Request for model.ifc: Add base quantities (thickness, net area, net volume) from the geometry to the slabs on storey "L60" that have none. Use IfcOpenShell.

First a look at what the model holds.

```python
import ifcopenshell
import ifcopenshell.util.element
import ifcopenshell.util.unit

model = ifcopenshell.open("model.ifc")
print(model.schema)
for unit_type in ("LENGTHUNIT", "AREAUNIT", "VOLUMEUNIT"):
    print(unit_type, ifcopenshell.util.unit.calculate_unit_scale(model, unit_type))
storey = next(s for s in model.by_type("IfcBuildingStorey") if s.Name == "L60")
slabs = [e for e in ifcopenshell.util.element.get_decomposition(storey) if e.is_a("IfcSlab")]
for e in sorted(slabs, key=lambda e: e.id()):
    print(e.id(), e.is_a(), e.Name, list(ifcopenshell.util.element.get_psets(e, qtos_only=True)), sep=" | ")
```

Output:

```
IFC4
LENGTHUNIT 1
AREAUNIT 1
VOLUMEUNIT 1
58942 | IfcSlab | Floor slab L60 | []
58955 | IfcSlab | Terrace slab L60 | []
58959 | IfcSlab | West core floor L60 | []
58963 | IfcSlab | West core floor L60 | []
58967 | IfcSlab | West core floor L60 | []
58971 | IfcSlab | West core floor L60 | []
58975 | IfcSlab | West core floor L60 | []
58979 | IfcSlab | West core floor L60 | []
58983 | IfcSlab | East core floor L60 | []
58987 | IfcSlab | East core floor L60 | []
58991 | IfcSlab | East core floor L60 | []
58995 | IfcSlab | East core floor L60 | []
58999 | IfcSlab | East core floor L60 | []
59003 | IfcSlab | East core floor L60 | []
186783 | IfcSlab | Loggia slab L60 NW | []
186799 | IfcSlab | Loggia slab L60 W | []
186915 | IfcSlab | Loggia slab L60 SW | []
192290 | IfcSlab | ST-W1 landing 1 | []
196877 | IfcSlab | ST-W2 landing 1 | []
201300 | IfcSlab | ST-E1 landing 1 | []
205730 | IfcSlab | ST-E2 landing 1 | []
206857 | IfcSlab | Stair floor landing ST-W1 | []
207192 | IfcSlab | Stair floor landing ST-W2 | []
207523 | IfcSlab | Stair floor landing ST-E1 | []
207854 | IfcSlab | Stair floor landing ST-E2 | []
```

```python
import ifcopenshell
import ifcopenshell.api.pset
import ifcopenshell.geom
import ifcopenshell.util.element
import ifcopenshell.util.shape
import ifcopenshell.util.unit

model = ifcopenshell.open("model.ifc")
unit_scale = ifcopenshell.util.unit.calculate_unit_scale(model)
area_scale = ifcopenshell.util.unit.calculate_unit_scale(model, "AREAUNIT")
volume_scale = ifcopenshell.util.unit.calculate_unit_scale(model, "VOLUMEUNIT")
settings = ifcopenshell.geom.settings()

storey = next(s for s in model.by_type("IfcBuildingStorey") if s.Name == "L60")
slabs = [e for e in ifcopenshell.util.element.get_decomposition(storey) if e.is_a("IfcSlab")]

for e in sorted(slabs, key=lambda e: e.id()):
    if ifcopenshell.util.element.get_psets(e, qtos_only=True, should_inherit=False):
        continue
    # Geometry comes back in metres, in the element's own axes.
    shape = ifcopenshell.geom.create_shape(settings, e)
    values = {
        "Width": ifcopenshell.util.shape.get_z(shape.geometry) / unit_scale,
        "NetArea": ifcopenshell.util.shape.get_footprint_area(shape.geometry) / area_scale,
        "NetVolume": ifcopenshell.util.shape.get_volume(shape.geometry) / volume_scale,
    }
    qto = ifcopenshell.api.pset.add_qto(model, product=e, name="Qto_SlabBaseQuantities")
    ifcopenshell.api.pset.edit_qto(model, qto=qto, properties=values)
    print(e.id(), {k: round(v, 3) for k, v in values.items()})

model.write("model_rev.ifc")
```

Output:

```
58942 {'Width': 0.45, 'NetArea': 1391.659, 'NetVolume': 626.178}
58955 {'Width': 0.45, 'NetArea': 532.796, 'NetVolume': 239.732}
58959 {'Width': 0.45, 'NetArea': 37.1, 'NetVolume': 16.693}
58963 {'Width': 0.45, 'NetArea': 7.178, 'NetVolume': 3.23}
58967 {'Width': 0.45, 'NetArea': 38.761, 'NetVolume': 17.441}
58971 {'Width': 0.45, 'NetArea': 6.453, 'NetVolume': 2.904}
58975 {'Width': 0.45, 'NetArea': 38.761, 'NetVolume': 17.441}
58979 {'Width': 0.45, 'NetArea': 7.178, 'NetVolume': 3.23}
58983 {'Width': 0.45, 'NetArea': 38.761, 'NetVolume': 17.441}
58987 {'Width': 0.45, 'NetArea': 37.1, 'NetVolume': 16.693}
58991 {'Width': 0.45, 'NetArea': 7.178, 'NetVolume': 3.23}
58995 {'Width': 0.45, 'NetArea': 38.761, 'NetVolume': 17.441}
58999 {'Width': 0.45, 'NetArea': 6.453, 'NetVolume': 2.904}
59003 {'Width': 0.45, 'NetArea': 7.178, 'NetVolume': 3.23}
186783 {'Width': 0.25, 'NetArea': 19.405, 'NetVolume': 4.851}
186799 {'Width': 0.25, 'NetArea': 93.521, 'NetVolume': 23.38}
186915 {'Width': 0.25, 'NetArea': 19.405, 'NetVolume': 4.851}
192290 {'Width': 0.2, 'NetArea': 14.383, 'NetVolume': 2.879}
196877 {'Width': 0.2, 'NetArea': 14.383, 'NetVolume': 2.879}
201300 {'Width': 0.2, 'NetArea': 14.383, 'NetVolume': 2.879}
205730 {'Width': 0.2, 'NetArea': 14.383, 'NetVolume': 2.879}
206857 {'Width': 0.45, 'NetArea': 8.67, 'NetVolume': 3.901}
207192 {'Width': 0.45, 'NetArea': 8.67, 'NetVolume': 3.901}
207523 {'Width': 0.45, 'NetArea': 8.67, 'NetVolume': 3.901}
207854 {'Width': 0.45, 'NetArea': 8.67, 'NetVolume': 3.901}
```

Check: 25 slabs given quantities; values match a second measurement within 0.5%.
